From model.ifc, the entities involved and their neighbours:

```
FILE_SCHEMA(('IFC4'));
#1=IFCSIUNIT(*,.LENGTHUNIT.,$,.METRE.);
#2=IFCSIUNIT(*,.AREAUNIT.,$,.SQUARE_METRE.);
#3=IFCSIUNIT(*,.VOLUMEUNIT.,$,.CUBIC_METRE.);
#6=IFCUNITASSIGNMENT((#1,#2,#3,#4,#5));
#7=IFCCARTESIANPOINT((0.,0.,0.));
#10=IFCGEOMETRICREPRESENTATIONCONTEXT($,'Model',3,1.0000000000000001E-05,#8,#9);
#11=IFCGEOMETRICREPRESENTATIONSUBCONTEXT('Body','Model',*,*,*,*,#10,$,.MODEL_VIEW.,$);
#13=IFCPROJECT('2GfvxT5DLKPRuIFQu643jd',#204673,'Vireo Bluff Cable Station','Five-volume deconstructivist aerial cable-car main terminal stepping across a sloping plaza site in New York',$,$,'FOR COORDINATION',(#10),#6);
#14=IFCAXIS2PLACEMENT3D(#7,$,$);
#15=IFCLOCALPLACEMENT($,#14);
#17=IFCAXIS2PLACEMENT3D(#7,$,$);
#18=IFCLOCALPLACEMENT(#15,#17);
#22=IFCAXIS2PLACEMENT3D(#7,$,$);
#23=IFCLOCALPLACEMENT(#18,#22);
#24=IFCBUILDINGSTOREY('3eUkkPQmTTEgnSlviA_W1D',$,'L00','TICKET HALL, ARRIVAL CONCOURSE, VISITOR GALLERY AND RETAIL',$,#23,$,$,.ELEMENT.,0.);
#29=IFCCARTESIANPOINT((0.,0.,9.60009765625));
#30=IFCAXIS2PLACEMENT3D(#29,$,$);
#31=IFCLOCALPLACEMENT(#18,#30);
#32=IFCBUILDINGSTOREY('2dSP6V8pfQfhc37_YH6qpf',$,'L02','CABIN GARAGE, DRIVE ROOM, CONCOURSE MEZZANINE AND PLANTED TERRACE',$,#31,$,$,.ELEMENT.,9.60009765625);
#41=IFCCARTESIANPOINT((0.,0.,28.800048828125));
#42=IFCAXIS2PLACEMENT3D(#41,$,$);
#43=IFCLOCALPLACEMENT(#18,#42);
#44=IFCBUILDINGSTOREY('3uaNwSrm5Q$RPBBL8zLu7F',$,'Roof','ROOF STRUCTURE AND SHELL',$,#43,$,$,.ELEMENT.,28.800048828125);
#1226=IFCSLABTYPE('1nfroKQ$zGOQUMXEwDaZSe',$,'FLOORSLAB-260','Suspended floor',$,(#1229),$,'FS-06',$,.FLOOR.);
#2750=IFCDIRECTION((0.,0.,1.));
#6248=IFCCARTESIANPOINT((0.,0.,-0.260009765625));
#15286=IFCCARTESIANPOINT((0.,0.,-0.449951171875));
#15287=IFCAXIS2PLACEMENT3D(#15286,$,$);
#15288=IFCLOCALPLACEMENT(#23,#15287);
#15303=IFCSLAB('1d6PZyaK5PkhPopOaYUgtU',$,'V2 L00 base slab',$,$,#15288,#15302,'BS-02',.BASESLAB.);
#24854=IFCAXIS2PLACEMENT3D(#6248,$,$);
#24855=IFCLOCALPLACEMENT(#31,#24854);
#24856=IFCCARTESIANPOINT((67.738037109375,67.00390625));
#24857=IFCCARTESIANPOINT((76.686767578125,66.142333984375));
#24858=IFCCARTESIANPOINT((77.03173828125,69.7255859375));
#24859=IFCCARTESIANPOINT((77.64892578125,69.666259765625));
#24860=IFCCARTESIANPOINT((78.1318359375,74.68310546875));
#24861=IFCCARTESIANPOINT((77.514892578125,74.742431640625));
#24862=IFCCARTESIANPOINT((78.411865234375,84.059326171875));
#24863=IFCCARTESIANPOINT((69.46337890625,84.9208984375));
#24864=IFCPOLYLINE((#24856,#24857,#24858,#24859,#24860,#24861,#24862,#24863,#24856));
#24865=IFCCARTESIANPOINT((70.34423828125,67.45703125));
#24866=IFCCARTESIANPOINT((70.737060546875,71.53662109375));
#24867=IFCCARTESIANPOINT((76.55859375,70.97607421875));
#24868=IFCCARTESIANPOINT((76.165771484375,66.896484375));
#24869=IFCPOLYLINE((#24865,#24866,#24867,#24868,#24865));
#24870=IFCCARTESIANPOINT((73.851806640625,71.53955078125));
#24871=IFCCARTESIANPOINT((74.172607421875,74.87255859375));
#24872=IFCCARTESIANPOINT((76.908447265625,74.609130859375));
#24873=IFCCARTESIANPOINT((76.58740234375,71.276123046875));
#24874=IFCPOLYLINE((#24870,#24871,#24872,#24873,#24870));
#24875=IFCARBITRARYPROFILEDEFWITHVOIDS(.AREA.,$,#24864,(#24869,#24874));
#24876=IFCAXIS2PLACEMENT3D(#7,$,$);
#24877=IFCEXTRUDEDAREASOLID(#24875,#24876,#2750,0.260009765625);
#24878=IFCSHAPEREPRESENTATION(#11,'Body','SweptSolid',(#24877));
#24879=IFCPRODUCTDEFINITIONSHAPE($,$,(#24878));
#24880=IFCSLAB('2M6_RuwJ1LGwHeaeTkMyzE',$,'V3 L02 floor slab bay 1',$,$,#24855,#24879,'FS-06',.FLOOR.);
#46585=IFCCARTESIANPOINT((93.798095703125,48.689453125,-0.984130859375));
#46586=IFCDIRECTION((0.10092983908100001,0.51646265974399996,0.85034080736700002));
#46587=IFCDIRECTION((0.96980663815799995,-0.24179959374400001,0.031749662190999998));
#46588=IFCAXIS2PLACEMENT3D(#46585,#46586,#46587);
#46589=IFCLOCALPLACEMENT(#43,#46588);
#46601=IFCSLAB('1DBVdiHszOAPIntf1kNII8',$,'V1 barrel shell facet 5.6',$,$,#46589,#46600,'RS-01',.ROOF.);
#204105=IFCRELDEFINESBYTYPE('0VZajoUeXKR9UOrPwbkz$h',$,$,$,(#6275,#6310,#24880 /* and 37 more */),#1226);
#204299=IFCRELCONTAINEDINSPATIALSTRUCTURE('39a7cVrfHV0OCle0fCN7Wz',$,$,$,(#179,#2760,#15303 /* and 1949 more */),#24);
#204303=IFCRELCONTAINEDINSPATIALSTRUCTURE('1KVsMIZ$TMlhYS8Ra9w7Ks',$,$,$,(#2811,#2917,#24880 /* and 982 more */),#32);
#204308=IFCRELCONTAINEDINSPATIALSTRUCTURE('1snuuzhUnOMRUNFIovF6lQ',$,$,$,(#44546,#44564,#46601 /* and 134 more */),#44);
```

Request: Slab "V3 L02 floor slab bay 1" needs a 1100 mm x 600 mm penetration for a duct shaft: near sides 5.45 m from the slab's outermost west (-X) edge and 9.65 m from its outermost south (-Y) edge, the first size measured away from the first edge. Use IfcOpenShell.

```python
import numpy as np
import ifcopenshell
import ifcopenshell.api.feature
import ifcopenshell.api.geometry
import ifcopenshell.api.root
import ifcopenshell.geom
import ifcopenshell.util.placement
import ifcopenshell.util.representation
import ifcopenshell.util.shape
import ifcopenshell.util.unit

model = ifcopenshell.open("model.ifc")
unit_scale = ifcopenshell.util.unit.calculate_unit_scale(model)
settings = ifcopenshell.geom.settings()


def volume(element):
    """Net volume in cubic metres, openings subtracted."""
    shape = ifcopenshell.geom.create_shape(settings, element)
    return ifcopenshell.util.shape.get_volume(shape.geometry)


slab = model.by_guid("2M6_RuwJ1LGwHeaeTkMyzE")
before = volume(slab)

# Extent in the slab's own axes, in metres. The edges named are its -X and -Y sides.
slab_shape = ifcopenshell.geom.create_shape(settings, slab)
vertices = ifcopenshell.util.shape.get_vertices(slab_shape.geometry)
x_min, y_min, bottom = vertices.min(axis=0)
top = vertices[:, 2].max()

opening = ifcopenshell.api.root.create_entity(model, ifc_class="IfcOpeningElement", name="Duct shaft opening", predefined_type="OPENING")
context = ifcopenshell.util.representation.get_context(model, "Model", "Body", "MODEL_VIEW")
width, depth = 1.1, 0.6
outline = [(0.0, 0.0), (width, 0.0), (width, depth), (0.0, depth), (0.0, 0.0)]
# Overshoot both faces by 50 mm so the cut is clean.
shape = ifcopenshell.api.geometry.add_slab_representation(
    model, context=context, depth=top - bottom + 0.1, polyline=outline
)
ifcopenshell.api.geometry.assign_representation(model, product=opening, representation=shape)

matrix = ifcopenshell.util.placement.get_local_placement(slab.ObjectPlacement)
matrix[:, 3] = matrix @ np.append(np.array([x_min + 5.45, y_min + 9.65, bottom - 0.05]) / unit_scale, 1.0)
ifcopenshell.api.geometry.edit_object_placement(model, product=opening, matrix=matrix, is_si=False)
ifcopenshell.api.feature.add_feature(model, feature=opening, element=slab)

after = volume(slab)

print(f"slab volume {before:.3f} -> {after:.3f} m3")

model.write("model_rev.ifc")
```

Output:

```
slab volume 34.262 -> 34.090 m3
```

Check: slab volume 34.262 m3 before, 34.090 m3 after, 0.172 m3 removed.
